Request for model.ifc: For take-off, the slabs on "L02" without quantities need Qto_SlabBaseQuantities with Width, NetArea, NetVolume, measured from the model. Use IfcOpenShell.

First a look at what the model holds.

```python
import ifcopenshell
import ifcopenshell.util.element
import ifcopenshell.util.unit

model = ifcopenshell.open("model.ifc")
print(model.schema)
for unit_type in ("LENGTHUNIT", "AREAUNIT", "VOLUMEUNIT"):
    print(unit_type, ifcopenshell.util.unit.calculate_unit_scale(model, unit_type))
storey = next(s for s in model.by_type("IfcBuildingStorey") if s.Name == "L02")
slabs = [e for e in ifcopenshell.util.element.get_decomposition(storey) if e.is_a("IfcSlab")]
for e in sorted(slabs, key=lambda e: e.id()):
    print(e.id(), e.is_a(), e.Name, list(ifcopenshell.util.element.get_psets(e, qtos_only=True)), sep=" | ")
```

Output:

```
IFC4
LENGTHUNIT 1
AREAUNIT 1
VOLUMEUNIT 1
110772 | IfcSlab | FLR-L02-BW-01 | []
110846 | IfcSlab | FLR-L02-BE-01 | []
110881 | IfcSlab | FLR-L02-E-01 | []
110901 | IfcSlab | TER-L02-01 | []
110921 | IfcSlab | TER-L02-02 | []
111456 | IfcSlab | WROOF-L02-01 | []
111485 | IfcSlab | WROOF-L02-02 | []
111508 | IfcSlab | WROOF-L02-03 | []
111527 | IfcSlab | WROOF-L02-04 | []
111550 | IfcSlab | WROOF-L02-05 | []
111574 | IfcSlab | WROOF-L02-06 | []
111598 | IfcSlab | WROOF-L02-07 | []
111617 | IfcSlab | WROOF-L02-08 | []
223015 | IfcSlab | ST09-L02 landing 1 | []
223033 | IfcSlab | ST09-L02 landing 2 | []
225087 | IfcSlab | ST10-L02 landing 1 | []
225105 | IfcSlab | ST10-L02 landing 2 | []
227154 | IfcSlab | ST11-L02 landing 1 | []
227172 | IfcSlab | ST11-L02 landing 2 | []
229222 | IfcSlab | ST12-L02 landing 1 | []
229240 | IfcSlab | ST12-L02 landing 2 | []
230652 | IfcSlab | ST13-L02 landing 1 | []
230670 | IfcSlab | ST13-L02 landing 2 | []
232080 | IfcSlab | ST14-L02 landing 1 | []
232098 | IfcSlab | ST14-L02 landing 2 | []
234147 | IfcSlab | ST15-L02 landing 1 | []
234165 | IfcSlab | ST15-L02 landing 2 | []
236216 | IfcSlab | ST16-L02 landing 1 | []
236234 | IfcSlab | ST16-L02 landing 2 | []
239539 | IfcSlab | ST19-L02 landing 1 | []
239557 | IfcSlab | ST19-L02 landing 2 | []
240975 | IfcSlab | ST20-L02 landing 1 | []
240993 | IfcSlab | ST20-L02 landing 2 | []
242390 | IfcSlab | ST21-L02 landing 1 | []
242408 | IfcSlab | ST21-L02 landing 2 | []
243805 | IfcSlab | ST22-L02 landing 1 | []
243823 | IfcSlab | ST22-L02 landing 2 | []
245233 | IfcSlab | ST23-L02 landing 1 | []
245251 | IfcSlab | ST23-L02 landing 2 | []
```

```python
import ifcopenshell
import ifcopenshell.api.pset
import ifcopenshell.geom
import ifcopenshell.util.element
import ifcopenshell.util.shape
import ifcopenshell.util.unit

model = ifcopenshell.open("model.ifc")
unit_scale = ifcopenshell.util.unit.calculate_unit_scale(model)
area_scale = ifcopenshell.util.unit.calculate_unit_scale(model, "AREAUNIT")
volume_scale = ifcopenshell.util.unit.calculate_unit_scale(model, "VOLUMEUNIT")
settings = ifcopenshell.geom.settings()

storey = next(s for s in model.by_type("IfcBuildingStorey") if s.Name == "L02")
slabs = [e for e in ifcopenshell.util.element.get_decomposition(storey) if e.is_a("IfcSlab")]

for e in sorted(slabs, key=lambda e: e.id()):
    if ifcopenshell.util.element.get_psets(e, qtos_only=True, should_inherit=False):
        continue
    # Geometry comes back in metres, in the element's own axes.
    shape = ifcopenshell.geom.create_shape(settings, e)
    values = {
        "Width": ifcopenshell.util.shape.get_z(shape.geometry) / unit_scale,
        "NetArea": ifcopenshell.util.shape.get_footprint_area(shape.geometry) / area_scale,
        "NetVolume": ifcopenshell.util.shape.get_volume(shape.geometry) / volume_scale,
    }
    qto = ifcopenshell.api.pset.add_qto(model, product=e, name="Qto_SlabBaseQuantities")
    ifcopenshell.api.pset.edit_qto(model, qto=qto, properties=values)
    print(e.id(), {k: round(v, 3) for k, v in values.items()})

model.write("model_edited.ifc")
```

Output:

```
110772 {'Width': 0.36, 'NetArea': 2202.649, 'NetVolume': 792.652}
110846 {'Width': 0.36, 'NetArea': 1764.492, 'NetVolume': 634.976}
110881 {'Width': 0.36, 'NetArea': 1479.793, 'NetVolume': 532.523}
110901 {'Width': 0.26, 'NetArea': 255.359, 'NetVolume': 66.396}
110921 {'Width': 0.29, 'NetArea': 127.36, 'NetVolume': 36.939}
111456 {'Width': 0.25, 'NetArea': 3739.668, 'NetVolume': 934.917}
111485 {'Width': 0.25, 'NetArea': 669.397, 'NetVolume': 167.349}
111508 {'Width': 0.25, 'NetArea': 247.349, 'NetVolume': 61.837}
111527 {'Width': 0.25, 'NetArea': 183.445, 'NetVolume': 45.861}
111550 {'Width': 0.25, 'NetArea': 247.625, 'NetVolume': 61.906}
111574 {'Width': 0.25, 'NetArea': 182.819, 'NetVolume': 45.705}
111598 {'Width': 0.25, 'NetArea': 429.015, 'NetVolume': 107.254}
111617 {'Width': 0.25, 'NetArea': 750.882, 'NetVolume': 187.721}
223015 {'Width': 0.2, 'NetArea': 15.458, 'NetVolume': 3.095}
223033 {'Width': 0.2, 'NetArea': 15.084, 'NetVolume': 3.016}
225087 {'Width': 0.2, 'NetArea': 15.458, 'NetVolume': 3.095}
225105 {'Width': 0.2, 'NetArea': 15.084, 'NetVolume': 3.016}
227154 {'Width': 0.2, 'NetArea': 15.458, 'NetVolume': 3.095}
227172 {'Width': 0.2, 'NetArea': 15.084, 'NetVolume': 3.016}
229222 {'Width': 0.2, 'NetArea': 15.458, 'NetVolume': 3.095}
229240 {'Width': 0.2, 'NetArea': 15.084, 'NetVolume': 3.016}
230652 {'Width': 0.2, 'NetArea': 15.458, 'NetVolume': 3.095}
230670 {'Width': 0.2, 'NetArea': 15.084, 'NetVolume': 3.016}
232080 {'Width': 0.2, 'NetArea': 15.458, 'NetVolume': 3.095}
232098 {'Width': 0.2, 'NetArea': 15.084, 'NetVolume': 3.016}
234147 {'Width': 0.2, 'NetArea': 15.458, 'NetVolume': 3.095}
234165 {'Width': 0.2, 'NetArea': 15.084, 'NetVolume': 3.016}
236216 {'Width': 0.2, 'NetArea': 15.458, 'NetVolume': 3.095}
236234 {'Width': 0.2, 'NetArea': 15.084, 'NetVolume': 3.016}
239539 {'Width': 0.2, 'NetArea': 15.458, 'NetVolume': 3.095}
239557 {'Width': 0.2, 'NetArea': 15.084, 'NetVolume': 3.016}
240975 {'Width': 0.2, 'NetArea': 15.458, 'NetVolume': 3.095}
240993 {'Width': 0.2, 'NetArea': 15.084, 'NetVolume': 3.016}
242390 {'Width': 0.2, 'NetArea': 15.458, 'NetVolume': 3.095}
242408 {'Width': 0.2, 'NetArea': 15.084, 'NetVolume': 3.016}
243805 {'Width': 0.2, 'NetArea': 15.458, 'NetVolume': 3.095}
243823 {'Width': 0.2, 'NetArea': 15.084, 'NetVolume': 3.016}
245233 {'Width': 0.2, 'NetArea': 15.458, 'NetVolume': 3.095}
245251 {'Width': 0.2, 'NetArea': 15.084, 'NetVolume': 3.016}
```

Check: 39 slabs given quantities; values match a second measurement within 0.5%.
